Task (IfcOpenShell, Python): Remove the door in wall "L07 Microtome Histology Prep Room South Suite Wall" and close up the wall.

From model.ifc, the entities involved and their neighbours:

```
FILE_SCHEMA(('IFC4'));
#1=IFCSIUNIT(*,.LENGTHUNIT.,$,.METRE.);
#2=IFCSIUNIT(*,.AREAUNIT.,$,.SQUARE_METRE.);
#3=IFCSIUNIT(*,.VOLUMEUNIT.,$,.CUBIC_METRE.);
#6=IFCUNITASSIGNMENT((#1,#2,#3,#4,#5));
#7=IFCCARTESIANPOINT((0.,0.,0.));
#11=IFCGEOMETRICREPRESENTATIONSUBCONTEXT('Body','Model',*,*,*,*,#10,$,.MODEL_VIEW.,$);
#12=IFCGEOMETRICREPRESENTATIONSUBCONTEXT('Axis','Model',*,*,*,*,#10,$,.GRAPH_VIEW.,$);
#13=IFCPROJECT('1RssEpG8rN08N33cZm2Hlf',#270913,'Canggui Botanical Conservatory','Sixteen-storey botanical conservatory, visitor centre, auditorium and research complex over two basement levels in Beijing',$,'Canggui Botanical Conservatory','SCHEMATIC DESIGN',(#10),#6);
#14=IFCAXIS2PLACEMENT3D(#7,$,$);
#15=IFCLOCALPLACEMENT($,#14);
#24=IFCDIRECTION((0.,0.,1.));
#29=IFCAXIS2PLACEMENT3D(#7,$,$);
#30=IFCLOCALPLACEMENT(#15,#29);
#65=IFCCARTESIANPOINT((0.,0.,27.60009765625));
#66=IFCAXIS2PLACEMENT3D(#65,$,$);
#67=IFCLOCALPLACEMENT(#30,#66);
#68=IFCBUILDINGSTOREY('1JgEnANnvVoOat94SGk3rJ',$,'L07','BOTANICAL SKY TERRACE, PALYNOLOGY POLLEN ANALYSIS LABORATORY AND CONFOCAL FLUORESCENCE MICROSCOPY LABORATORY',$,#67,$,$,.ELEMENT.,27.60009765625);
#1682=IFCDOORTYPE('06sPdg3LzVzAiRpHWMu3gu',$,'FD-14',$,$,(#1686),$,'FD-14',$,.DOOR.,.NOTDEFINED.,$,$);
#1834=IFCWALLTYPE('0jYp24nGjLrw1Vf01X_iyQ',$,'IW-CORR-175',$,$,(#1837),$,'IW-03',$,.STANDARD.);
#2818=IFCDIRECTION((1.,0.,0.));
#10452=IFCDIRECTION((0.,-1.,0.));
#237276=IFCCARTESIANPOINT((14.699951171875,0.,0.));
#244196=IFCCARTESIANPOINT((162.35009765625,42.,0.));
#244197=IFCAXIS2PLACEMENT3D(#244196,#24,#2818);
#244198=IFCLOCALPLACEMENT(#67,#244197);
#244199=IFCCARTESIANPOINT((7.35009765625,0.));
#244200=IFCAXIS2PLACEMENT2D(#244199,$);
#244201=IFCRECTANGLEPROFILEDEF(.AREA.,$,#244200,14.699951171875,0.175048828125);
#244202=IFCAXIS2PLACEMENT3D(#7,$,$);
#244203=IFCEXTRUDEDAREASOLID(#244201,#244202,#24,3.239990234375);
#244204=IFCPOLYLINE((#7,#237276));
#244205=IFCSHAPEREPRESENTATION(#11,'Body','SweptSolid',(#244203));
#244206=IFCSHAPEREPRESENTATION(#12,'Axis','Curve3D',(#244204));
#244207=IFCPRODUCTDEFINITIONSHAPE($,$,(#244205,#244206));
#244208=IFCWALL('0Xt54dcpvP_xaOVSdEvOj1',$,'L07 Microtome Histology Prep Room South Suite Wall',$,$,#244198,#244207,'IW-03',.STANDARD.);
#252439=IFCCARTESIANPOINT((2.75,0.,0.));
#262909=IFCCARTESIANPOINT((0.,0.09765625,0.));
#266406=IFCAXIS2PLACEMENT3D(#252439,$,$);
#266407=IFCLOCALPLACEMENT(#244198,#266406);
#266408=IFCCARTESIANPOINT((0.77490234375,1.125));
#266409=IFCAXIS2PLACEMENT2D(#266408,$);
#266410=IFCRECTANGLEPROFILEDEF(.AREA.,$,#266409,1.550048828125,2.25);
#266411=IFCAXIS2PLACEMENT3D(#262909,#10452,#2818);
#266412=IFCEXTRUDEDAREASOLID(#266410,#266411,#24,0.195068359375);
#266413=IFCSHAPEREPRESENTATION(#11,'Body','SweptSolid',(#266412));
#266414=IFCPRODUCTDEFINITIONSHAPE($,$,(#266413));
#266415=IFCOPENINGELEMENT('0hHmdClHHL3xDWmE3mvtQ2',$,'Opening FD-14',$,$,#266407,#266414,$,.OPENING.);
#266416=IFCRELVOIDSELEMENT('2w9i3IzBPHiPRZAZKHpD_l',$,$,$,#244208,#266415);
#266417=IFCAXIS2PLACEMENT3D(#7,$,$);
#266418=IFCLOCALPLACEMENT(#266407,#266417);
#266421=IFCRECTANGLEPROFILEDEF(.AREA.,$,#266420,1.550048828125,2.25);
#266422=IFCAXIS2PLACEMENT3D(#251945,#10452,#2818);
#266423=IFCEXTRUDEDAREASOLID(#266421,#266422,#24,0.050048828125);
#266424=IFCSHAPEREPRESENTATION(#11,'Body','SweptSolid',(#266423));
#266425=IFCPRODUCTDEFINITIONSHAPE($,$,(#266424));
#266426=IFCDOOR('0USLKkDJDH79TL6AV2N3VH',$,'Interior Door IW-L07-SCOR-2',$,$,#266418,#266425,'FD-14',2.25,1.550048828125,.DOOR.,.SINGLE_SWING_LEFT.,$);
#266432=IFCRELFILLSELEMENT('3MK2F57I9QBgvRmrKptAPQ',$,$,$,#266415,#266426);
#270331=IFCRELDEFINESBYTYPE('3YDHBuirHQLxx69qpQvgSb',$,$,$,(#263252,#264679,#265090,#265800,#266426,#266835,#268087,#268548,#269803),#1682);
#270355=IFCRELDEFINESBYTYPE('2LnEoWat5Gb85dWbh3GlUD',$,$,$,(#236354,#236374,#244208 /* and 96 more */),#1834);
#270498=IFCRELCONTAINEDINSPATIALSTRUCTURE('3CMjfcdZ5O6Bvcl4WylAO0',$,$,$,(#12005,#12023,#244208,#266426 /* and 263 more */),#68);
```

```python
import ifcopenshell
import ifcopenshell.api.feature
import ifcopenshell.api.root
import ifcopenshell.geom
import ifcopenshell.util.shape

model = ifcopenshell.open("model.ifc")
settings = ifcopenshell.geom.settings()


def volume(element):
    """Net volume in cubic metres, openings subtracted."""
    shape = ifcopenshell.geom.create_shape(settings, element)
    return ifcopenshell.util.shape.get_volume(shape.geometry)


door = model.by_guid("0USLKkDJDH79TL6AV2N3VH")
opening = door.FillsVoids[0].RelatingOpeningElement
wall = opening.VoidsElements[0].RelatingBuildingElement
before = volume(wall)

ifcopenshell.api.root.remove_product(model, product=door)
ifcopenshell.api.feature.remove_feature(model, feature=opening)

after = volume(wall)

print(f"wall volume {before:.3f} -> {after:.3f} m3")

model.write("model_v2.ifc")
```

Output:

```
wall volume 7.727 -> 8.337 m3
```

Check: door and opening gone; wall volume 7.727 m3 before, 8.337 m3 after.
